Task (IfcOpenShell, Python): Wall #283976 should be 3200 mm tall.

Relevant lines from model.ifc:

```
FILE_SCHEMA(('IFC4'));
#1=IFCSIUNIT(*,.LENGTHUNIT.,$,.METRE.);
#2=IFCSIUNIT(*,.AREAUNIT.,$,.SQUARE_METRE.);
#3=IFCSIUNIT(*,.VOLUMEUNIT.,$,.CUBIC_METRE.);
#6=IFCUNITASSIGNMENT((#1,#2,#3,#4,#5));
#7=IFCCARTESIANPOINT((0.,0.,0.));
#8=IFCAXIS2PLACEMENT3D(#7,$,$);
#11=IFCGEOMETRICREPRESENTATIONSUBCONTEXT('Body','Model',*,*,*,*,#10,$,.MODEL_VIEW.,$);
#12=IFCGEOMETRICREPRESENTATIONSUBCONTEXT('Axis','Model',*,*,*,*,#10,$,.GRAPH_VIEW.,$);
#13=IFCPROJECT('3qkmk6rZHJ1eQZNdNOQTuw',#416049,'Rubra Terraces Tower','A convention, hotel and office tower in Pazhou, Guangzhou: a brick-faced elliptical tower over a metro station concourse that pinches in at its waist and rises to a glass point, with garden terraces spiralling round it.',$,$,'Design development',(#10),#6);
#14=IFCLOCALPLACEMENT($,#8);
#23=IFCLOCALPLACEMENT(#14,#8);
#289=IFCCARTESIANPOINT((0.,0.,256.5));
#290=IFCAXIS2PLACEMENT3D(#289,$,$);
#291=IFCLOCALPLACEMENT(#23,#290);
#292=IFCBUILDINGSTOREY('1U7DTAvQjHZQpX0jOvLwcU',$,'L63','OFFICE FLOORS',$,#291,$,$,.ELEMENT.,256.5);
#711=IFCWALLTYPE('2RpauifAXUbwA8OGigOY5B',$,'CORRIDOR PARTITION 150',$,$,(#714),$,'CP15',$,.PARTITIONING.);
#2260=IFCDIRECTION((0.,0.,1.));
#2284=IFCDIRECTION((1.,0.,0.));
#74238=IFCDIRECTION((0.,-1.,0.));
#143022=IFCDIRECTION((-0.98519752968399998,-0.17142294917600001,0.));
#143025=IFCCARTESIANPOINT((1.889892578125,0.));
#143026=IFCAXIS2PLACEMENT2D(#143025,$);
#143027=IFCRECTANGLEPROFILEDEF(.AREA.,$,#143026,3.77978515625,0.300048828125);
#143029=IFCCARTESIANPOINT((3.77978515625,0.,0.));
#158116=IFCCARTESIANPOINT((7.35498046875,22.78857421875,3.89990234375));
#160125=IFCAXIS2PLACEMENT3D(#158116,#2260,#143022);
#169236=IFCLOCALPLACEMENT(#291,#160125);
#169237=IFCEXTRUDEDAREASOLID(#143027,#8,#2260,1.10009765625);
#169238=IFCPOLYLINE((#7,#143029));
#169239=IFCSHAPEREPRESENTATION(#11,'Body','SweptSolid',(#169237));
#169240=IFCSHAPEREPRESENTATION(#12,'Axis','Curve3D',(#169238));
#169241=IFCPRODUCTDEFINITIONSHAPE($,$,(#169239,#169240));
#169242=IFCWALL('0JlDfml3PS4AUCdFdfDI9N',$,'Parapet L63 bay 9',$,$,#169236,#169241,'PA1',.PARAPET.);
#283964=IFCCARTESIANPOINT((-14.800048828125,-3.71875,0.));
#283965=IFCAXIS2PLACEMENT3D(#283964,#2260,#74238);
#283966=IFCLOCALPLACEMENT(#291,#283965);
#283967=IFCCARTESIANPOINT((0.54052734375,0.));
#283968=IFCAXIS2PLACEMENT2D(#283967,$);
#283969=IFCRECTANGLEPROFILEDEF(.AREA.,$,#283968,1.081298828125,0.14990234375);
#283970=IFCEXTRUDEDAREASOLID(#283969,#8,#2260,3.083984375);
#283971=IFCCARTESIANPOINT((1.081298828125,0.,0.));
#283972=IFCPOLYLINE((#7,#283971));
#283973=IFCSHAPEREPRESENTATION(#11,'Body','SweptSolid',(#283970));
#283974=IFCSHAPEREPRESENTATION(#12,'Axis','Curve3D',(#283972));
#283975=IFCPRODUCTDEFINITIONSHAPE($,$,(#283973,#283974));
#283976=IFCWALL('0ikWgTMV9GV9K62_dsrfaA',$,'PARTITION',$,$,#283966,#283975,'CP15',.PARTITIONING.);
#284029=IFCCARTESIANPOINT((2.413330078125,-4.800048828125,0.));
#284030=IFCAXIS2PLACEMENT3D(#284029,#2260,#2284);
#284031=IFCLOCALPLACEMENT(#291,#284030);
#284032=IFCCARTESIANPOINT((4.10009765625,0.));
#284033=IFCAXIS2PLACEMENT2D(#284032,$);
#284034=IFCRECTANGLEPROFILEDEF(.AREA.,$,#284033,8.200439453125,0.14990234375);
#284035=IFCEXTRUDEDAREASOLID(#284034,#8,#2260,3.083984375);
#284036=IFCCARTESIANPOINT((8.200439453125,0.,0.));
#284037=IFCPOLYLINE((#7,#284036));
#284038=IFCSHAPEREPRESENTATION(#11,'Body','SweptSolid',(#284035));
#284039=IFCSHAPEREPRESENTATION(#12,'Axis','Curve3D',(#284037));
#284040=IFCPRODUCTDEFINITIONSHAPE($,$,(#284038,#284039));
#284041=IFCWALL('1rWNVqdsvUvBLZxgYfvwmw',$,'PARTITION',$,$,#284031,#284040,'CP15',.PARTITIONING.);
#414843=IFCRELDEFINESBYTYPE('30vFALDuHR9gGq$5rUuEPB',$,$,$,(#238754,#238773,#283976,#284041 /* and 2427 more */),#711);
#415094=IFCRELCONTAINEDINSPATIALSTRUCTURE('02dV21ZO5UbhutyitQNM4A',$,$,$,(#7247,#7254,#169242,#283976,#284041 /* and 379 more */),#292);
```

```python
import ifcopenshell
import ifcopenshell.geom
import ifcopenshell.util.representation
import ifcopenshell.util.shape

model = ifcopenshell.open("model.ifc")
settings = ifcopenshell.geom.settings()


def volume(element):
    """Net volume in cubic metres, openings subtracted."""
    shape = ifcopenshell.geom.create_shape(settings, element)
    return ifcopenshell.util.shape.get_volume(shape.geometry)


wall = model.by_id(283976)
before = volume(wall)

body = ifcopenshell.util.representation.get_representation(wall, "Model", "Body")
solid = body.Items[0]
old_height = solid.Depth
solid.Depth = 3.2
after = volume(wall)

print(f"height {old_height:g} -> {solid.Depth:g}, volume {before:.3f} -> {after:.3f} m3")

model.write("model_updated.ifc")
```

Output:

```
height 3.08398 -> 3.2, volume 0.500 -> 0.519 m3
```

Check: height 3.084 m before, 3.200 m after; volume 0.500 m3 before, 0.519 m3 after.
